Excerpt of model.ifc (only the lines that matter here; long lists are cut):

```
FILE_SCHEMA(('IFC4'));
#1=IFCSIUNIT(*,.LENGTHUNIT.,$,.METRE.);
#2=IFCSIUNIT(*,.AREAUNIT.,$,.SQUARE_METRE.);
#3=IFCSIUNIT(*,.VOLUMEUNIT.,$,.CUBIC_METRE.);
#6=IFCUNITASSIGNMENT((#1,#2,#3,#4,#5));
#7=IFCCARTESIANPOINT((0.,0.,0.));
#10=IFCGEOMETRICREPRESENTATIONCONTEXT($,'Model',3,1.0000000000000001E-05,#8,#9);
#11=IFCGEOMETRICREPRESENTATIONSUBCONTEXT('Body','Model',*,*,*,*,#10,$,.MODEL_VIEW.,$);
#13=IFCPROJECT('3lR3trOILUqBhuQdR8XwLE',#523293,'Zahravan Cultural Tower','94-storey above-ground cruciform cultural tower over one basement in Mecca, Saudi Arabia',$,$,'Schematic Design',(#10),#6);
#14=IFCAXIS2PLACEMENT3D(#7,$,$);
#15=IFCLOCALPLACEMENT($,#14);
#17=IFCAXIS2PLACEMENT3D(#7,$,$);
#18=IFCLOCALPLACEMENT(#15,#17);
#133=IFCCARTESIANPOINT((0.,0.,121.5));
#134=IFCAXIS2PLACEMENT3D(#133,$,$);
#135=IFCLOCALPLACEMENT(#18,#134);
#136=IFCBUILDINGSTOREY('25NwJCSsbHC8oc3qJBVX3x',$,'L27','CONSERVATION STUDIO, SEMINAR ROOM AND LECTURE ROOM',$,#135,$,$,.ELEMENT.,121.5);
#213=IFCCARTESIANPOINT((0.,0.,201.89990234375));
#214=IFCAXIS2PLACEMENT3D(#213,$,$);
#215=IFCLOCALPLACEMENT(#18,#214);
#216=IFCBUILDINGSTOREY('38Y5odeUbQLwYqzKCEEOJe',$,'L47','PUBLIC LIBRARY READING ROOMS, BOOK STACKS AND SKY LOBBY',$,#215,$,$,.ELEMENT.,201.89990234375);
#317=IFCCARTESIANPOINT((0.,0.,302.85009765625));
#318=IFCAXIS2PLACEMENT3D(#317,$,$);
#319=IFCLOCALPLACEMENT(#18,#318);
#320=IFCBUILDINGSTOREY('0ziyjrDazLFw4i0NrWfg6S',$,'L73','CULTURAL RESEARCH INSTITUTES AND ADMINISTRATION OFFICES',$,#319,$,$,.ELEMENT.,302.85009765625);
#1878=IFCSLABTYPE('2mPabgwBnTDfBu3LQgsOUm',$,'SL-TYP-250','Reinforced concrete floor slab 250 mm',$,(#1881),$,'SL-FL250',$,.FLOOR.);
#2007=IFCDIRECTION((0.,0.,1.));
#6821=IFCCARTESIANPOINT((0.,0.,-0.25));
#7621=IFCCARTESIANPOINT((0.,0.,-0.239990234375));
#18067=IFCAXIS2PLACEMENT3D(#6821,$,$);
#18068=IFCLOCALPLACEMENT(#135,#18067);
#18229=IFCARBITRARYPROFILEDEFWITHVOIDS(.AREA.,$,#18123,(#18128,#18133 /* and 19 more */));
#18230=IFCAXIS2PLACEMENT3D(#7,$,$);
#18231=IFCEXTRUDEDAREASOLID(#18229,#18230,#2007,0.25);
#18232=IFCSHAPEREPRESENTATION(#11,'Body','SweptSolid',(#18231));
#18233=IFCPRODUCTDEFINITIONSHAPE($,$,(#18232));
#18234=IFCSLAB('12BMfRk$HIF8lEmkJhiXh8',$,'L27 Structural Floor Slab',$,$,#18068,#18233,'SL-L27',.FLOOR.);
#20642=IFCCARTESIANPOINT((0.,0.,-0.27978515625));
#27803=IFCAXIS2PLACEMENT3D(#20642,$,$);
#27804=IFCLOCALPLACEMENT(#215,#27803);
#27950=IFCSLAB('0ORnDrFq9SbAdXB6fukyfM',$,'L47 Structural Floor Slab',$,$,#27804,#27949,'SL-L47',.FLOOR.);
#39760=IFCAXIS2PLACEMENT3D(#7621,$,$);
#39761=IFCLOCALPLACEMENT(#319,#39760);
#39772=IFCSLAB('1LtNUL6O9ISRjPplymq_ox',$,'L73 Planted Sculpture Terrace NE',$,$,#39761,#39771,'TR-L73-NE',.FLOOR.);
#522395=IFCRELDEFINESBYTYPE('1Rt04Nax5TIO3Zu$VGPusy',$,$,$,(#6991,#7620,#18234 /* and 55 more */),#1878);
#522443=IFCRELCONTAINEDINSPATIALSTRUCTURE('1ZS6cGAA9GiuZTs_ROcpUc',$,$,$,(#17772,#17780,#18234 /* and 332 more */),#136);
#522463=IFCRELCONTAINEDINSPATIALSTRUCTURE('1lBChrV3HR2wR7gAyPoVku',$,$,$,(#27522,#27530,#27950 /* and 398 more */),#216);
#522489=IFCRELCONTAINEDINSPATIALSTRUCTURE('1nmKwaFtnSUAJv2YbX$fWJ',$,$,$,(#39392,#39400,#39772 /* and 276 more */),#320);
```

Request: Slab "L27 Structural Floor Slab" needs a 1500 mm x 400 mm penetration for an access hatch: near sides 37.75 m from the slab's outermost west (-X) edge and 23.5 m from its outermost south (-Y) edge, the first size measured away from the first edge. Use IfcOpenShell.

```python
import numpy as np
import ifcopenshell
import ifcopenshell.api.feature
import ifcopenshell.api.geometry
import ifcopenshell.api.root
import ifcopenshell.geom
import ifcopenshell.util.placement
import ifcopenshell.util.representation
import ifcopenshell.util.shape
import ifcopenshell.util.unit

model = ifcopenshell.open("model.ifc")
unit_scale = ifcopenshell.util.unit.calculate_unit_scale(model)
settings = ifcopenshell.geom.settings()


def volume(element):
    """Net volume in cubic metres, openings subtracted."""
    shape = ifcopenshell.geom.create_shape(settings, element)
    return ifcopenshell.util.shape.get_volume(shape.geometry)


slab = model.by_id(18234)
before = volume(slab)

# Extent in the slab's own axes, in metres. The edges named are its -X and -Y sides.
slab_shape = ifcopenshell.geom.create_shape(settings, slab)
vertices = ifcopenshell.util.shape.get_vertices(slab_shape.geometry)
x_min, y_min, bottom = vertices.min(axis=0)
top = vertices[:, 2].max()

opening = ifcopenshell.api.root.create_entity(model, ifc_class="IfcOpeningElement", name="Access hatch opening", predefined_type="OPENING")
context = ifcopenshell.util.representation.get_context(model, "Model", "Body", "MODEL_VIEW")
width, depth = 1.5, 0.4
outline = [(0.0, 0.0), (width, 0.0), (width, depth), (0.0, depth), (0.0, 0.0)]
# Overshoot both faces by 50 mm so the cut is clean.
shape = ifcopenshell.api.geometry.add_slab_representation(
    model, context=context, depth=top - bottom + 0.1, polyline=outline
)
ifcopenshell.api.geometry.assign_representation(model, product=opening, representation=shape)

matrix = ifcopenshell.util.placement.get_local_placement(slab.ObjectPlacement)
matrix[:, 3] = matrix @ np.append(np.array([x_min + 37.75, y_min + 23.5, bottom - 0.05]) / unit_scale, 1.0)
ifcopenshell.api.geometry.edit_object_placement(model, product=opening, matrix=matrix, is_si=False)
ifcopenshell.api.feature.add_feature(model, feature=opening, element=slab)

after = volume(slab)

print(f"slab volume {before:.3f} -> {after:.3f} m3")

model.write("model_v2.ifc")
```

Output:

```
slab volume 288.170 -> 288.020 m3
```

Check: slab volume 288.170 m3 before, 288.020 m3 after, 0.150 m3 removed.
